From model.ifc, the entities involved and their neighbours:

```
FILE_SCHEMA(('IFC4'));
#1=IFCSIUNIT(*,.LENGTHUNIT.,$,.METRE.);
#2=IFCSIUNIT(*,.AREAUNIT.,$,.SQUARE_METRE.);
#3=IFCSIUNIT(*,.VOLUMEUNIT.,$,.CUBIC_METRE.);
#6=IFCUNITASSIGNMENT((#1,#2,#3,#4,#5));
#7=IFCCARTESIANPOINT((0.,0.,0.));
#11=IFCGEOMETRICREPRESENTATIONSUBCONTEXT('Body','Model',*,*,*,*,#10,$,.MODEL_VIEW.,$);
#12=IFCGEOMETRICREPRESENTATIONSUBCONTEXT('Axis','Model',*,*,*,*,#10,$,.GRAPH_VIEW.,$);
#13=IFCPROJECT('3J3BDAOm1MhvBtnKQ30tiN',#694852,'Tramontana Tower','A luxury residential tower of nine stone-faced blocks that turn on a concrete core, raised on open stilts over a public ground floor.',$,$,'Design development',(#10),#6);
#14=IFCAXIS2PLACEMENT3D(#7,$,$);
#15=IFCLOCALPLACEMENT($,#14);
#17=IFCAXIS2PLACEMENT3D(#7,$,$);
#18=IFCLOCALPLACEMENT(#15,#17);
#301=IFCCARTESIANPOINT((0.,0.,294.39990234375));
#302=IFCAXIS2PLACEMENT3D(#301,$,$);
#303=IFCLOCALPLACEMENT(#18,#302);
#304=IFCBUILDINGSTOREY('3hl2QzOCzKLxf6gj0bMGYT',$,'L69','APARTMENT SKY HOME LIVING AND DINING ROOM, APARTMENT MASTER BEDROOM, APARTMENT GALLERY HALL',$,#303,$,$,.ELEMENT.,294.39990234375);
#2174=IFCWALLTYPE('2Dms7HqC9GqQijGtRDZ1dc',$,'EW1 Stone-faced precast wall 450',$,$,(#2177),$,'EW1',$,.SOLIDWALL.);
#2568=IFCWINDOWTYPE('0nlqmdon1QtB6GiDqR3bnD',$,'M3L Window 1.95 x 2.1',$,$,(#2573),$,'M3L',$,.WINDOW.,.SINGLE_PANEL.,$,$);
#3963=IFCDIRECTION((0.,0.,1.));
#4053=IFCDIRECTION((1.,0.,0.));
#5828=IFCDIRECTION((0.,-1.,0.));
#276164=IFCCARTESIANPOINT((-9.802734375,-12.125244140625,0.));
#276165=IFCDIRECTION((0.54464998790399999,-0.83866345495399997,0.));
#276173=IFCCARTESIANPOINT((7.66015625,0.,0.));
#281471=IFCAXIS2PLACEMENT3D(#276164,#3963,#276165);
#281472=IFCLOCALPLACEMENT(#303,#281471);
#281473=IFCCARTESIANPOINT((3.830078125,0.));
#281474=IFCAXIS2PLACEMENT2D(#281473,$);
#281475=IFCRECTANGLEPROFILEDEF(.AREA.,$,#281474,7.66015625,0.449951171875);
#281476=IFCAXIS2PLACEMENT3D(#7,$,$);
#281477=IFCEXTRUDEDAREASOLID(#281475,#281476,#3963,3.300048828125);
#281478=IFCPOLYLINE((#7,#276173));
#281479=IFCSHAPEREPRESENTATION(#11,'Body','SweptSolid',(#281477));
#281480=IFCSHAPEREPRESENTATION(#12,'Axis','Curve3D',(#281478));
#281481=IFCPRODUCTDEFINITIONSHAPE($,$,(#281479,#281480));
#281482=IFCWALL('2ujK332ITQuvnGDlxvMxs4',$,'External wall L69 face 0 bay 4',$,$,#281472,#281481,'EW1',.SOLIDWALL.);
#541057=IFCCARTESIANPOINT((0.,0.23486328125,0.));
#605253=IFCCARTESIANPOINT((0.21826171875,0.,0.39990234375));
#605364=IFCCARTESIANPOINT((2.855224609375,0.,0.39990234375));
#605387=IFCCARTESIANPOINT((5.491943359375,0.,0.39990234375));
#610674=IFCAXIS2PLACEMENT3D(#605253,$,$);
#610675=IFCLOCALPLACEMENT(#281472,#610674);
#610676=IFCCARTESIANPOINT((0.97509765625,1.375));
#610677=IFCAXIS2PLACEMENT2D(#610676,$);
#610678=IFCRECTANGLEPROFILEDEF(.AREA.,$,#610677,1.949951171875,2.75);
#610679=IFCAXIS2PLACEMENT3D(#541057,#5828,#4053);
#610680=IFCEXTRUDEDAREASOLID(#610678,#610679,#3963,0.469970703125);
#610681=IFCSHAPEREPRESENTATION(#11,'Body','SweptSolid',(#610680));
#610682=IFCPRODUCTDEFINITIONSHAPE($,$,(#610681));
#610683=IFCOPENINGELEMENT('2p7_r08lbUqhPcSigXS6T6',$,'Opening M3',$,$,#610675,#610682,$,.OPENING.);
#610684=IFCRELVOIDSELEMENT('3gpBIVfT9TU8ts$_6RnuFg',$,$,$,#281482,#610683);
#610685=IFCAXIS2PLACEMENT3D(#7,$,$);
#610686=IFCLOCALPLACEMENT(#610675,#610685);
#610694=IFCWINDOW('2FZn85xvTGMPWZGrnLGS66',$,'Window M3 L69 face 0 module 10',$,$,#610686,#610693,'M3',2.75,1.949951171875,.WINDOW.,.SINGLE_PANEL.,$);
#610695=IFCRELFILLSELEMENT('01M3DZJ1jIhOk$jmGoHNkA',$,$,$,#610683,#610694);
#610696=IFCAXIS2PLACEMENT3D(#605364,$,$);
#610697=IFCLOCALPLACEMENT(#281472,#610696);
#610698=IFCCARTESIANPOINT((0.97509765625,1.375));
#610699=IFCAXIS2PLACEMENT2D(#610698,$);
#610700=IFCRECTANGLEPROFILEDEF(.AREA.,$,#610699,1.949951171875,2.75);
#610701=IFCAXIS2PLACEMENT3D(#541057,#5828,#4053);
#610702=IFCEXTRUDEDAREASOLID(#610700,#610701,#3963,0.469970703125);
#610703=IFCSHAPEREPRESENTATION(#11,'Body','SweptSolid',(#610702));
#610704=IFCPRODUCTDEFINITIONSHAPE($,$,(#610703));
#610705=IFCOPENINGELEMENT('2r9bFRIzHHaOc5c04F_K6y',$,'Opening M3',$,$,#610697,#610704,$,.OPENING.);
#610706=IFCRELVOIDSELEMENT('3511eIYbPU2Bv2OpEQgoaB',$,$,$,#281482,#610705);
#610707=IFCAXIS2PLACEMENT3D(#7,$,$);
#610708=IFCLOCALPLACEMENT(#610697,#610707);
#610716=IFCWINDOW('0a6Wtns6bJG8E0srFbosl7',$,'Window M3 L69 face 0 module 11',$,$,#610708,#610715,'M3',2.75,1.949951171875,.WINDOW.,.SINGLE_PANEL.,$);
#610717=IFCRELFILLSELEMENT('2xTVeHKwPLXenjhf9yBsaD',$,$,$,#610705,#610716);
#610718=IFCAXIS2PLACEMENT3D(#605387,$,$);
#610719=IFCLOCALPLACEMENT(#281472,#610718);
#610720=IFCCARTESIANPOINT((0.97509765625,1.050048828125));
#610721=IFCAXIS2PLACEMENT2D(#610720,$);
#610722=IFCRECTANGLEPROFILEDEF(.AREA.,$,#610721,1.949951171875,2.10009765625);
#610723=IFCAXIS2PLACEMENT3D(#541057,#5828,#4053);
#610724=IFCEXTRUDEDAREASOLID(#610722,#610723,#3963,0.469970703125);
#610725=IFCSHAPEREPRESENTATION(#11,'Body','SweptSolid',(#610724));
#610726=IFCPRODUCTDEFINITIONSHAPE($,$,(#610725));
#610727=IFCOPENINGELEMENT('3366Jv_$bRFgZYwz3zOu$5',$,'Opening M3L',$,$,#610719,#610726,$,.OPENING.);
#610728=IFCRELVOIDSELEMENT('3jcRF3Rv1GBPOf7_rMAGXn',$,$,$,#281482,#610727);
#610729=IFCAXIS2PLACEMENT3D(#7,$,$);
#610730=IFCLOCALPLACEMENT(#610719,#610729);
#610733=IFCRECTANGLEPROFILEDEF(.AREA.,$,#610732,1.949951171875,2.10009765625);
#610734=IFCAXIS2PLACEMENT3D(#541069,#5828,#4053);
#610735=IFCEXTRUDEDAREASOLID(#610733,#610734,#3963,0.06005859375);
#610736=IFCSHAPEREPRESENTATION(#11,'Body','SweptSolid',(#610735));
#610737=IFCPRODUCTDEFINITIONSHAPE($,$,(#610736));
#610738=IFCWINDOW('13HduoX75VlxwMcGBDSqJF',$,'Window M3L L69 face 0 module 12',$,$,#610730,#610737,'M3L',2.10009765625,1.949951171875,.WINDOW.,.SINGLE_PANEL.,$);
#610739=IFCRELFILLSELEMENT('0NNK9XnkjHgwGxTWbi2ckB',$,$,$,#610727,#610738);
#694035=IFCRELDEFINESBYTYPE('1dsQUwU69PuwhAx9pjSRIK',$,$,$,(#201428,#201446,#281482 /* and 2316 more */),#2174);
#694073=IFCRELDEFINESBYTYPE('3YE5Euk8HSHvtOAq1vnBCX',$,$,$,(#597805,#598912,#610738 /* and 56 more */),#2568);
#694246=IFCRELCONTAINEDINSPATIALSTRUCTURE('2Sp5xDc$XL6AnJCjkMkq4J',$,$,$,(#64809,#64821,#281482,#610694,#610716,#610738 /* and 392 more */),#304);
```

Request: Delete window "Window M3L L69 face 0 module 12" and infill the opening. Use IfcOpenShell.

```python
import ifcopenshell
import ifcopenshell.api.feature
import ifcopenshell.api.root
import ifcopenshell.geom
import ifcopenshell.util.shape

model = ifcopenshell.open("model.ifc")
settings = ifcopenshell.geom.settings()


def volume(element):
    """Net volume in cubic metres, openings subtracted."""
    shape = ifcopenshell.geom.create_shape(settings, element)
    return ifcopenshell.util.shape.get_volume(shape.geometry)


window = model.by_id(610738)
opening = window.FillsVoids[0].RelatingOpeningElement
wall = opening.VoidsElements[0].RelatingBuildingElement
before = volume(wall)

ifcopenshell.api.root.remove_product(model, product=window)
ifcopenshell.api.feature.remove_feature(model, feature=opening)

after = volume(wall)

print(f"wall volume {before:.3f} -> {after:.3f} m3")

model.write("model_updated.ifc")
```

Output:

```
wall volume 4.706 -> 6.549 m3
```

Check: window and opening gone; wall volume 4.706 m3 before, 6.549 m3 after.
